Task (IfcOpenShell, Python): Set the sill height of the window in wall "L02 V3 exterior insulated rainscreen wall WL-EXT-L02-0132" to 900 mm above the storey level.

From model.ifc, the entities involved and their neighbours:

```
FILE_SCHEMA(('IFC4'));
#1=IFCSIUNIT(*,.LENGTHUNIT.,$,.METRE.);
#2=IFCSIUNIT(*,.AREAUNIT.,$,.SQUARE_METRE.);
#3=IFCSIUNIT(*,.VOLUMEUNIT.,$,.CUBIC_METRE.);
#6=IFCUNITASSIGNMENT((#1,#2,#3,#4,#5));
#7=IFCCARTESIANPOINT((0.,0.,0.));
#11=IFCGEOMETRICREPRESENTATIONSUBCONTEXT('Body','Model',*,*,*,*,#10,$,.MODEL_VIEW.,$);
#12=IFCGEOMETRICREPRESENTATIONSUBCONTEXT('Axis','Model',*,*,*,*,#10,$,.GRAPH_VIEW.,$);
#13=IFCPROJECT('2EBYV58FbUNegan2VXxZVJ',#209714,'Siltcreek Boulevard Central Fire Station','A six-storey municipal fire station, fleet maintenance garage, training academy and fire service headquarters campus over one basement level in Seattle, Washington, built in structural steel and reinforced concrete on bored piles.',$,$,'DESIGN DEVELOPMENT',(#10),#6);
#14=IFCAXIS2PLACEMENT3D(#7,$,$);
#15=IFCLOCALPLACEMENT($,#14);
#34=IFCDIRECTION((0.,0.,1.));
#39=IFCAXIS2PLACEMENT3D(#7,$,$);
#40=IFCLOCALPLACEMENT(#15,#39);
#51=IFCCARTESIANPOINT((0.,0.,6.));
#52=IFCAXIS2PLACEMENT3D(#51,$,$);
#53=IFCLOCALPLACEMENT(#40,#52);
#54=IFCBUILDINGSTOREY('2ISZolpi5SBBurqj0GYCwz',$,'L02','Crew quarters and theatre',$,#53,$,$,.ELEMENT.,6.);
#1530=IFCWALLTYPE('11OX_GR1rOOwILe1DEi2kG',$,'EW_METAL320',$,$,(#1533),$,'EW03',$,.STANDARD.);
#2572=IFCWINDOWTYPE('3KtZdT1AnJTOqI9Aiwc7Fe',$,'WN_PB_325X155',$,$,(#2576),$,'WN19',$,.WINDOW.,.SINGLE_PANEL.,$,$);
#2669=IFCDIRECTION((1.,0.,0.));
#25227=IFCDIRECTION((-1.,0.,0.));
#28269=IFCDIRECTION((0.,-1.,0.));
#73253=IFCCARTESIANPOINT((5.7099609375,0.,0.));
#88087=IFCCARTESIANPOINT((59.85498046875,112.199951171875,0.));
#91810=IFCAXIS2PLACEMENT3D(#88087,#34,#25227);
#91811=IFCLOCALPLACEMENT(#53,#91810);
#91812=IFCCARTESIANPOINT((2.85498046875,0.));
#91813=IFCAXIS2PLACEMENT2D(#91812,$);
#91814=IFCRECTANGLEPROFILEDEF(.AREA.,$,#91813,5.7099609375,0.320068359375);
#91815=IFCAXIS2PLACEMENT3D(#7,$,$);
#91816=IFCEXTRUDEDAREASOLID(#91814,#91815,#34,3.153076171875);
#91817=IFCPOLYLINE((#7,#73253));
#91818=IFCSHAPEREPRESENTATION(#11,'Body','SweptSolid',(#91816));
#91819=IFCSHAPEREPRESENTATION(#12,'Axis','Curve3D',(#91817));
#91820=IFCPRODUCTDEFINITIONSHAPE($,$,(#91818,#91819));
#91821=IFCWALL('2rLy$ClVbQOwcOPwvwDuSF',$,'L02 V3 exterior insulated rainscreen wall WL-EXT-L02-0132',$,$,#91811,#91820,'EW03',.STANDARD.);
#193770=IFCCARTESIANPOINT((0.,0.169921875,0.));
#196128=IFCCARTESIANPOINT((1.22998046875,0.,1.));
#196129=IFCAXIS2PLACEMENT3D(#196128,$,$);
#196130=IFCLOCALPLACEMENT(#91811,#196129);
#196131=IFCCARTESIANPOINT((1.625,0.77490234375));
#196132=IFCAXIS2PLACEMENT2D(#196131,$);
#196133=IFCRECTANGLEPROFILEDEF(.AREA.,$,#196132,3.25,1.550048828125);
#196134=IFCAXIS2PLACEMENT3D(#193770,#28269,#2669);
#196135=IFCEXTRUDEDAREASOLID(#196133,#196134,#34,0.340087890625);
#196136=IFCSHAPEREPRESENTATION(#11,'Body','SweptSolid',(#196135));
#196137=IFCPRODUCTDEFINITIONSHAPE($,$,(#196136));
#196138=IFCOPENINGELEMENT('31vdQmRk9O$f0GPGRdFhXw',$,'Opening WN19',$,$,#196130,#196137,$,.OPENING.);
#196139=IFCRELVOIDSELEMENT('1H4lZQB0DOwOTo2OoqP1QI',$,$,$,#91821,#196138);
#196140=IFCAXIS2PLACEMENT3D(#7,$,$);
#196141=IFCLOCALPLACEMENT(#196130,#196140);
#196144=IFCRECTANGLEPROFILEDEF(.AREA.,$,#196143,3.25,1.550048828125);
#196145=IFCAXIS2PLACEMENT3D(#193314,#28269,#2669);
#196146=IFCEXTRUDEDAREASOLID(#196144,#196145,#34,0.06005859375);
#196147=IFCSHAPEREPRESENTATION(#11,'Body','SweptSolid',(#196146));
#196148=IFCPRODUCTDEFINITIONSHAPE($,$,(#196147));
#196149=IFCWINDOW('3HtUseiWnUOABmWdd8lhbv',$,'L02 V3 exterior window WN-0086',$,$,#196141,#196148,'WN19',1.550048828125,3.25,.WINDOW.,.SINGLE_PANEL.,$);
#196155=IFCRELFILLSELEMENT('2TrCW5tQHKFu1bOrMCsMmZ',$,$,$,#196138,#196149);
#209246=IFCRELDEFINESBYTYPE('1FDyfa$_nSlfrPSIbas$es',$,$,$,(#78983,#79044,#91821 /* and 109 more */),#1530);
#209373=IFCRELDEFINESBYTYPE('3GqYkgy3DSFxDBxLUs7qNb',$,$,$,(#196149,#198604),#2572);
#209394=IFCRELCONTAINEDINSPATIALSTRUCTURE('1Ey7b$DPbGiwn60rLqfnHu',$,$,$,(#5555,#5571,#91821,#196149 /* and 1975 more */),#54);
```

```python
import numpy as np
import ifcopenshell
import ifcopenshell.api.geometry
import ifcopenshell.geom
import ifcopenshell.util.element
import ifcopenshell.util.placement
import ifcopenshell.util.shape
import ifcopenshell.util.unit

model = ifcopenshell.open("model.ifc")
unit_scale = ifcopenshell.util.unit.calculate_unit_scale(model)

window = model.by_guid("3HtUseiWnUOABmWdd8lhbv")
opening = window.FillsVoids[0].RelatingOpeningElement
storey = ifcopenshell.util.element.get_container(window, ifc_class="IfcBuildingStorey")
level = ifcopenshell.util.placement.get_local_placement(storey.ObjectPlacement)[2, 3]

# The opening's origin need not be at the sill, so measure its lowest point.
shape = ifcopenshell.geom.create_shape(ifcopenshell.geom.settings(), opening)
bottom = ifcopenshell.util.shape.get_shape_bottom_elevation(shape, shape.geometry) / unit_scale
dz = level + 0.9 / unit_scale - bottom

shift = np.array([0.0, 0.0, dz])
# The window is placed relative to its opening, so it follows when the opening moves.
matrix = ifcopenshell.util.placement.get_local_placement(opening.ObjectPlacement)
matrix[:3, 3] += shift
ifcopenshell.api.geometry.edit_object_placement(
    model, product=opening, matrix=matrix, is_si=False, should_transform_children=True
)

print(f"moved by {dz * unit_scale:+.3f} m")

model.write("model-out.ifc")
```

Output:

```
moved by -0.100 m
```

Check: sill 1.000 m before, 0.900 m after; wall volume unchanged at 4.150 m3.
